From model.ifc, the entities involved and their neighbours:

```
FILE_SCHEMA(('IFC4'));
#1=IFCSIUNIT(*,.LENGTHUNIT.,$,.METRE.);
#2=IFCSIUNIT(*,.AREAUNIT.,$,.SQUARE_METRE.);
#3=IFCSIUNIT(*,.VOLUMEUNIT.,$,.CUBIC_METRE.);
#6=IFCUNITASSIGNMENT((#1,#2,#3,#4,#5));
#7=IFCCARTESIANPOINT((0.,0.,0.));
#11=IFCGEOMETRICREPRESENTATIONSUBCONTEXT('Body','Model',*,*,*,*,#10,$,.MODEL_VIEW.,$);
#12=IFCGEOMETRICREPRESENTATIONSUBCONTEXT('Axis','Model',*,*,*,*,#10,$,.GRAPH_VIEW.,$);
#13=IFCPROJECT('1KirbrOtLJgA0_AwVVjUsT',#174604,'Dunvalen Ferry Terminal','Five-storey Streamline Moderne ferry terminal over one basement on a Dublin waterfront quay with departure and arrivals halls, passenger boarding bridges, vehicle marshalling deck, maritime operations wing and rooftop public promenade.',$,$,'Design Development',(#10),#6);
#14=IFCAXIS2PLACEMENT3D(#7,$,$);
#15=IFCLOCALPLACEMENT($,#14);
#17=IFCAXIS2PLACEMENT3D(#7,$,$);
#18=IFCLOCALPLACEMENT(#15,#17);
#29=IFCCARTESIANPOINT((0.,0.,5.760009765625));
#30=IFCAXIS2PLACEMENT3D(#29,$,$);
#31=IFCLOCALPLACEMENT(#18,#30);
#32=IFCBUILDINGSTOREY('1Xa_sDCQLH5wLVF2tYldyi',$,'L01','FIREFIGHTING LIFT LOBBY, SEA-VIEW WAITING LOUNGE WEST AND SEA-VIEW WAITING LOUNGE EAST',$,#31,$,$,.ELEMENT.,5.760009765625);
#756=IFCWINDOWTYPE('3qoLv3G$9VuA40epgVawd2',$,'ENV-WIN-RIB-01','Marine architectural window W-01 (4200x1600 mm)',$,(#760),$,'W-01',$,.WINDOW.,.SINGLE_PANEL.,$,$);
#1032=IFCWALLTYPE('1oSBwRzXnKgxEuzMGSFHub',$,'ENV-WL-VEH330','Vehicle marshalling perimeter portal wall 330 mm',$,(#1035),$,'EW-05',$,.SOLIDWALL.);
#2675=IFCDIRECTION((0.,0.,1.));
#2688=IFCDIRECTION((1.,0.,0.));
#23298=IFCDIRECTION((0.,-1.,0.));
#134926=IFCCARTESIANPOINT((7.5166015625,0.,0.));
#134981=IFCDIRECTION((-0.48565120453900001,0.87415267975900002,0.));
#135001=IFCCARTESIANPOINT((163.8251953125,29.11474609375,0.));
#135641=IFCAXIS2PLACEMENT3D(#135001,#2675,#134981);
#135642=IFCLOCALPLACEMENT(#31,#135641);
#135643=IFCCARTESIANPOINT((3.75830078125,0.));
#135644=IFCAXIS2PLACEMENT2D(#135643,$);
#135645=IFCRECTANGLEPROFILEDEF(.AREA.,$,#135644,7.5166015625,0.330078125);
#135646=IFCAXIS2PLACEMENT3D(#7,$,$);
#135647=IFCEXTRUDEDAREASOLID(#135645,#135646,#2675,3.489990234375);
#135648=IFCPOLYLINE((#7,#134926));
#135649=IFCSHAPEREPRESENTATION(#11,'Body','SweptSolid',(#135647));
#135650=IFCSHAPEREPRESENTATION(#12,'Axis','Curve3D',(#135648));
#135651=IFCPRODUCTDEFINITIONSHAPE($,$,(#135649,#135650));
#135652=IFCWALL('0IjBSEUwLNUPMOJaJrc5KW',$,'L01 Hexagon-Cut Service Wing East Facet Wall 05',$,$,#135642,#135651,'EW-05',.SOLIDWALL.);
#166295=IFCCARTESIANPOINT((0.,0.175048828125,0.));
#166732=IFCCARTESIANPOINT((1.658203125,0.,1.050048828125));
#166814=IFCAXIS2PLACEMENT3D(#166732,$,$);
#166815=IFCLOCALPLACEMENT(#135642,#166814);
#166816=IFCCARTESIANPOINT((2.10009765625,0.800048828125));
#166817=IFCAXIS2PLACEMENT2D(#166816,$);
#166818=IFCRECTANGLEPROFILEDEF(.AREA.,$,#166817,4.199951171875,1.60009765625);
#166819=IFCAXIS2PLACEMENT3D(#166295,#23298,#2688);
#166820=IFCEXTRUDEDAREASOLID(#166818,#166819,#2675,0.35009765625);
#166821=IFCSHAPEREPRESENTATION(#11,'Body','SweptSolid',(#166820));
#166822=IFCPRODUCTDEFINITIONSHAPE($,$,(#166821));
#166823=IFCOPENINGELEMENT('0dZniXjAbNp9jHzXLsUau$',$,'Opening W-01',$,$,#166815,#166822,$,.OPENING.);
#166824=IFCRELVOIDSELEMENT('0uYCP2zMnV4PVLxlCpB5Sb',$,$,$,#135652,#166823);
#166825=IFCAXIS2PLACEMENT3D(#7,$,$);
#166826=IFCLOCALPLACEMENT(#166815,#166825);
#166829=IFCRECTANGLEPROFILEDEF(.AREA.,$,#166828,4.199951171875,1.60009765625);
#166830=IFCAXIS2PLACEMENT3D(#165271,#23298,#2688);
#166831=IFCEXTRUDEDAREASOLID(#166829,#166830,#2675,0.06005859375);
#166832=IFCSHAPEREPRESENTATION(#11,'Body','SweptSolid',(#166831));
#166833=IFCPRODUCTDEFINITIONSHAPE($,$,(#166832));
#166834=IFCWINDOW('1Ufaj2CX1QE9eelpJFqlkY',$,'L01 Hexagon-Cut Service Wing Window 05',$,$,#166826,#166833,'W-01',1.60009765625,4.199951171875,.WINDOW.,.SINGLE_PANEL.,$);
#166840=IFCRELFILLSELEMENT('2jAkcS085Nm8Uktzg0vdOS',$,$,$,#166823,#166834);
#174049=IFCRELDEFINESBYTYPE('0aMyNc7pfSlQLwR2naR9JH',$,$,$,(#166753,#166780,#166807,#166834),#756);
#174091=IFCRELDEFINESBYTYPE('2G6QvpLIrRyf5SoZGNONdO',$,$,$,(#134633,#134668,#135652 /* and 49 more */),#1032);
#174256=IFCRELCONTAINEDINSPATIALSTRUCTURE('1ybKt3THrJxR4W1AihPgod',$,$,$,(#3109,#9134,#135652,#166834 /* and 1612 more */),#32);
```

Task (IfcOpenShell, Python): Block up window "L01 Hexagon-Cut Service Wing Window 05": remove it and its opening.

```python
import ifcopenshell
import ifcopenshell.api.feature
import ifcopenshell.api.root
import ifcopenshell.geom
import ifcopenshell.util.shape

model = ifcopenshell.open("model.ifc")
settings = ifcopenshell.geom.settings()


def volume(element):
    """Net volume in cubic metres, openings subtracted."""
    shape = ifcopenshell.geom.create_shape(settings, element)
    return ifcopenshell.util.shape.get_volume(shape.geometry)


window = model.by_guid("1Ufaj2CX1QE9eelpJFqlkY")
opening = window.FillsVoids[0].RelatingOpeningElement
wall = opening.VoidsElements[0].RelatingBuildingElement
before = volume(wall)

ifcopenshell.api.root.remove_product(model, product=window)
ifcopenshell.api.feature.remove_feature(model, feature=opening)

after = volume(wall)

print(f"wall volume {before:.3f} -> {after:.3f} m3")

model.write("model_updated.ifc")
```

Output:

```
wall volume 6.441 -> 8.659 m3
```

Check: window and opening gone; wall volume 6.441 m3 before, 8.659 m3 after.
